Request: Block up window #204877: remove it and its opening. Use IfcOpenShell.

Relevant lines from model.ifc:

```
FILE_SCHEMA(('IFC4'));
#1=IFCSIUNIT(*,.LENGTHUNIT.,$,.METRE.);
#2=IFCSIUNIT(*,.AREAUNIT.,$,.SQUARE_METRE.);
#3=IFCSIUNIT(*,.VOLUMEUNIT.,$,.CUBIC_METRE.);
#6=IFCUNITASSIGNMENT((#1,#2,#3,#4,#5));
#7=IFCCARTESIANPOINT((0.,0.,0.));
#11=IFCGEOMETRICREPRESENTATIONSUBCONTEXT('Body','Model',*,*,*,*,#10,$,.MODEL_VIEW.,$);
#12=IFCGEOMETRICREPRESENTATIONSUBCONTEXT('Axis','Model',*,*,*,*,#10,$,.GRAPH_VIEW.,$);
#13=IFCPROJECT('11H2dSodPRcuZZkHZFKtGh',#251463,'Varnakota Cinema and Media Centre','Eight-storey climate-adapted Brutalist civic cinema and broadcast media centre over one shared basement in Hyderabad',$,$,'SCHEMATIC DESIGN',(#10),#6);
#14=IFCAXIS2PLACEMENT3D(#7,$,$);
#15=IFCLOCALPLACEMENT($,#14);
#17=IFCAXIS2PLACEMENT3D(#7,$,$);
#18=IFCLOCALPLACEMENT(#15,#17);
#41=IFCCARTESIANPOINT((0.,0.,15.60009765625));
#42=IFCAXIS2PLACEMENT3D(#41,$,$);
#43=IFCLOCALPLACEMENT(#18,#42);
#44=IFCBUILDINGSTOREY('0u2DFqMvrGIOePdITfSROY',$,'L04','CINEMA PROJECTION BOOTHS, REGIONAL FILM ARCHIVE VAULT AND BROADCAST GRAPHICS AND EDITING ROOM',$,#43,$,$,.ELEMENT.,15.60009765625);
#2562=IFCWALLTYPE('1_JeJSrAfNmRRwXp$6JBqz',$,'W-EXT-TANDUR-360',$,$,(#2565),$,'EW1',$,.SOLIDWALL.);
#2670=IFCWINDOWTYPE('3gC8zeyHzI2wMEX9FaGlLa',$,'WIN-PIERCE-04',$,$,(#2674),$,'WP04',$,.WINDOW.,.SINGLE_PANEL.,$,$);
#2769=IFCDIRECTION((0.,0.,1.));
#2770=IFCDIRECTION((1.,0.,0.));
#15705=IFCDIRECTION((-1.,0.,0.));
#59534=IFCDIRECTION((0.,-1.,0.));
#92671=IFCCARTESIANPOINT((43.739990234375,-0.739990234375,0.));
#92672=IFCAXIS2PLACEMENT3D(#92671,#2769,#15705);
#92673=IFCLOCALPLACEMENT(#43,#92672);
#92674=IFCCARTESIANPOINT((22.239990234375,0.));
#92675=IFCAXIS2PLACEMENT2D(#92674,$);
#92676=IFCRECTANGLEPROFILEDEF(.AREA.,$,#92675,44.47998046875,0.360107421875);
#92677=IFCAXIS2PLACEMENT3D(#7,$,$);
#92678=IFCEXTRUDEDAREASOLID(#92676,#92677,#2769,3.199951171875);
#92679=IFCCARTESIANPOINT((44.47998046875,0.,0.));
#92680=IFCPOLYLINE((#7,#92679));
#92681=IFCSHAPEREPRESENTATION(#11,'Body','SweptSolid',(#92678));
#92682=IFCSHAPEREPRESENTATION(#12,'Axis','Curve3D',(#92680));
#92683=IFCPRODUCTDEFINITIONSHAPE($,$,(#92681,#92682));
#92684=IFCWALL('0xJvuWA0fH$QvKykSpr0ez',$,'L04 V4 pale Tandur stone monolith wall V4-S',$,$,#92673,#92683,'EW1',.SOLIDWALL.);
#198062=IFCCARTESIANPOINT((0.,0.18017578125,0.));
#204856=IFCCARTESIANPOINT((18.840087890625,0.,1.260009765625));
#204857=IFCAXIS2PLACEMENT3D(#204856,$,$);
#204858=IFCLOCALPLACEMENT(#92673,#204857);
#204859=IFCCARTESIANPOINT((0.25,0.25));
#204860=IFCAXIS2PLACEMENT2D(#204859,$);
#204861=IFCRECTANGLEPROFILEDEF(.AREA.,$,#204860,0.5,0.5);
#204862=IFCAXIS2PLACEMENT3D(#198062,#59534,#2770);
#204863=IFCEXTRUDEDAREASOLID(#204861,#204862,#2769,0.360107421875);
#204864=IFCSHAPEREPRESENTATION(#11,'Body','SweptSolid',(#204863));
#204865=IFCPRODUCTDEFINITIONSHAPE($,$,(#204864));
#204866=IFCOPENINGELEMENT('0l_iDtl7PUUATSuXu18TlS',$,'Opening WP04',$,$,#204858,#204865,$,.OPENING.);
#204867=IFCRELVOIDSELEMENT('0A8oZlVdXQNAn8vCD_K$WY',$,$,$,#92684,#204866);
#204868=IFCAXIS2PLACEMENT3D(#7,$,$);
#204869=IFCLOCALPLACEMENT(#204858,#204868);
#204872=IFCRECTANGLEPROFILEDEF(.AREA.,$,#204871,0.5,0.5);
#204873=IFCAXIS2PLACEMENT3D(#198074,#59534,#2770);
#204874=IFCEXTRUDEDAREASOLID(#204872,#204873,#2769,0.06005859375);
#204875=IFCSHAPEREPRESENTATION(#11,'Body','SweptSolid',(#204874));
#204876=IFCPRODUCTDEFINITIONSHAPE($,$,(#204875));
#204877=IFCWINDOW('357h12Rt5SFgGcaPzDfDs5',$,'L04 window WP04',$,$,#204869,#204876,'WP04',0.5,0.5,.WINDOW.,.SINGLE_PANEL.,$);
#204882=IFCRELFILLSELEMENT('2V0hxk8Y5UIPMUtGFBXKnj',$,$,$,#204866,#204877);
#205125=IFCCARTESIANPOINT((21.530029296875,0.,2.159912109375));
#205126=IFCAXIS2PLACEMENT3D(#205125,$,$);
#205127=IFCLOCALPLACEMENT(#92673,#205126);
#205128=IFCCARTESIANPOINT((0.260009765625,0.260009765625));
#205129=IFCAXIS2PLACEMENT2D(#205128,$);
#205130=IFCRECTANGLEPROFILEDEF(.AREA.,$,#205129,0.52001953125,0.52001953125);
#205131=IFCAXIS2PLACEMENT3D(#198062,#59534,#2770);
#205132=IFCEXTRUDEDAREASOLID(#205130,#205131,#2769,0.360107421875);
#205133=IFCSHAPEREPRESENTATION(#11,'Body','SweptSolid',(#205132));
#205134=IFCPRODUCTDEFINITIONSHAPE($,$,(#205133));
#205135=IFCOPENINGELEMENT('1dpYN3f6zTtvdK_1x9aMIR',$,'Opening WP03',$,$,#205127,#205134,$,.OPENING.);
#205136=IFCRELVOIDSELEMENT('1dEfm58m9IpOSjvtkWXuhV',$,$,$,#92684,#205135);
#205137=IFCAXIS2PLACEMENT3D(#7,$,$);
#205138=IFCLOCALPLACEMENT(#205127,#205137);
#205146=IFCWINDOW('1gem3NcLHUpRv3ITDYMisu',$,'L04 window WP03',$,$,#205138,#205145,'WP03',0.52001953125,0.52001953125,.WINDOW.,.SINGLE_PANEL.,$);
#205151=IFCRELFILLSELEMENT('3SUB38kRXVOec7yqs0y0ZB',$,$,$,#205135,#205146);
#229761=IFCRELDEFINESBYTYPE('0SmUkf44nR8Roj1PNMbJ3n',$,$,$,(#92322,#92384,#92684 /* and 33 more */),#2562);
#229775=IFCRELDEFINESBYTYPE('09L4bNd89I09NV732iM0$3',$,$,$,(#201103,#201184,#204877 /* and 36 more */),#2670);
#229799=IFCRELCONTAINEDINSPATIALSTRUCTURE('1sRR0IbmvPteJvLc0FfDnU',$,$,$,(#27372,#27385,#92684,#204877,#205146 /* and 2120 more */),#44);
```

```python
import ifcopenshell
import ifcopenshell.api.feature
import ifcopenshell.api.root
import ifcopenshell.geom
import ifcopenshell.util.shape

model = ifcopenshell.open("model.ifc")
settings = ifcopenshell.geom.settings()


def volume(element):
    """Net volume in cubic metres, openings subtracted."""
    shape = ifcopenshell.geom.create_shape(settings, element)
    return ifcopenshell.util.shape.get_volume(shape.geometry)


window = model.by_id(204877)
opening = window.FillsVoids[0].RelatingOpeningElement
wall = opening.VoidsElements[0].RelatingBuildingElement
before = volume(wall)

ifcopenshell.api.root.remove_product(model, product=window)
ifcopenshell.api.feature.remove_feature(model, feature=opening)

after = volume(wall)

print(f"wall volume {before:.3f} -> {after:.3f} m3")

model.write("model_v2.ifc")
```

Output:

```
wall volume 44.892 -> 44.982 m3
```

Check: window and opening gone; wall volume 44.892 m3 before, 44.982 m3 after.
